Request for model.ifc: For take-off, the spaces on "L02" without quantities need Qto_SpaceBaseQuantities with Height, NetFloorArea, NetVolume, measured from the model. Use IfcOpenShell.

First a look at what the model holds.

```python
import ifcopenshell
import ifcopenshell.util.element
import ifcopenshell.util.unit

model = ifcopenshell.open("model.ifc")
print(model.schema)
for unit_type in ("LENGTHUNIT", "AREAUNIT", "VOLUMEUNIT"):
    print(unit_type, ifcopenshell.util.unit.calculate_unit_scale(model, unit_type))
storey = next(s for s in model.by_type("IfcBuildingStorey") if s.Name == "L02")
spaces = [e for e in ifcopenshell.util.element.get_decomposition(storey) if e.is_a("IfcSpace")]
for e in sorted(spaces, key=lambda e: e.id()):
    print(e.id(), e.is_a(), e.Name, list(ifcopenshell.util.element.get_psets(e, qtos_only=True)), sep=" | ")
```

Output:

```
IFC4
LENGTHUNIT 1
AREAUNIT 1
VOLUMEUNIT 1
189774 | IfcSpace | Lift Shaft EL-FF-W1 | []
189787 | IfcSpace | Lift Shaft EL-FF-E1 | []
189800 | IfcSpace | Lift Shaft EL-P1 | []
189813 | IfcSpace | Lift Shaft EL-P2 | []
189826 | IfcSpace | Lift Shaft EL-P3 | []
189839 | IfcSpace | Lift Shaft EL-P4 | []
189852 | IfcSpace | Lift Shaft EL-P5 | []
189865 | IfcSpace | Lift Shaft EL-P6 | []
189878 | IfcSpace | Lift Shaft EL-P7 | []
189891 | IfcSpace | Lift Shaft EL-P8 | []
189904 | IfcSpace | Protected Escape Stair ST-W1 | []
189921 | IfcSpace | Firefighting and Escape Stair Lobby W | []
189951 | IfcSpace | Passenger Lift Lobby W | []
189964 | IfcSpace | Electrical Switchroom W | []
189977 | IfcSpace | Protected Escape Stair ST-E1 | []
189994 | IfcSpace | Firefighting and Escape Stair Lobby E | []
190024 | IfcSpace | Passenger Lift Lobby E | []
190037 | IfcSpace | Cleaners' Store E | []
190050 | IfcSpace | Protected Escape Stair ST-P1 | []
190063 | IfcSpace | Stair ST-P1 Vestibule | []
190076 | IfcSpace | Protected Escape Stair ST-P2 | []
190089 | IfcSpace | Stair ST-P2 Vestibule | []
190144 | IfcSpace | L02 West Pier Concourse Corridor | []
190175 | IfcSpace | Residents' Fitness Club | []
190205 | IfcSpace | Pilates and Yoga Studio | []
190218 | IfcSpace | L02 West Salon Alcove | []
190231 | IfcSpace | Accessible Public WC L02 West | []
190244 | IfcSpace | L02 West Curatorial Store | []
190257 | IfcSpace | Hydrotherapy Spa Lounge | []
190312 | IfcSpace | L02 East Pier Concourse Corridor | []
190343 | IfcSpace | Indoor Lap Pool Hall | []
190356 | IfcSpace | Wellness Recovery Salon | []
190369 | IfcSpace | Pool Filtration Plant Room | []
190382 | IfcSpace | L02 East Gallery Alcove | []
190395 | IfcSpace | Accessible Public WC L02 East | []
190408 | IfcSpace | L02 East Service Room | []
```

```python
import ifcopenshell
import ifcopenshell.api.pset
import ifcopenshell.geom
import ifcopenshell.util.element
import ifcopenshell.util.shape
import ifcopenshell.util.unit

model = ifcopenshell.open("model.ifc")
unit_scale = ifcopenshell.util.unit.calculate_unit_scale(model)
area_scale = ifcopenshell.util.unit.calculate_unit_scale(model, "AREAUNIT")
volume_scale = ifcopenshell.util.unit.calculate_unit_scale(model, "VOLUMEUNIT")
settings = ifcopenshell.geom.settings()

storey = next(s for s in model.by_type("IfcBuildingStorey") if s.Name == "L02")
spaces = [e for e in ifcopenshell.util.element.get_decomposition(storey) if e.is_a("IfcSpace")]

for e in sorted(spaces, key=lambda e: e.id()):
    if ifcopenshell.util.element.get_psets(e, qtos_only=True, should_inherit=False):
        continue
    # Geometry comes back in metres, in the element's own axes.
    shape = ifcopenshell.geom.create_shape(settings, e)
    values = {
        "Height": ifcopenshell.util.shape.get_z(shape.geometry) / unit_scale,
        "NetFloorArea": ifcopenshell.util.shape.get_footprint_area(shape.geometry) / area_scale,
        "NetVolume": ifcopenshell.util.shape.get_volume(shape.geometry) / volume_scale,
    }
    qto = ifcopenshell.api.pset.add_qto(model, product=e, name="Qto_SpaceBaseQuantities")
    ifcopenshell.api.pset.edit_qto(model, qto=qto, properties=values)
    print(e.id(), {k: round(v, 3) for k, v in values.items()})

model.write("model_edited.ifc")
```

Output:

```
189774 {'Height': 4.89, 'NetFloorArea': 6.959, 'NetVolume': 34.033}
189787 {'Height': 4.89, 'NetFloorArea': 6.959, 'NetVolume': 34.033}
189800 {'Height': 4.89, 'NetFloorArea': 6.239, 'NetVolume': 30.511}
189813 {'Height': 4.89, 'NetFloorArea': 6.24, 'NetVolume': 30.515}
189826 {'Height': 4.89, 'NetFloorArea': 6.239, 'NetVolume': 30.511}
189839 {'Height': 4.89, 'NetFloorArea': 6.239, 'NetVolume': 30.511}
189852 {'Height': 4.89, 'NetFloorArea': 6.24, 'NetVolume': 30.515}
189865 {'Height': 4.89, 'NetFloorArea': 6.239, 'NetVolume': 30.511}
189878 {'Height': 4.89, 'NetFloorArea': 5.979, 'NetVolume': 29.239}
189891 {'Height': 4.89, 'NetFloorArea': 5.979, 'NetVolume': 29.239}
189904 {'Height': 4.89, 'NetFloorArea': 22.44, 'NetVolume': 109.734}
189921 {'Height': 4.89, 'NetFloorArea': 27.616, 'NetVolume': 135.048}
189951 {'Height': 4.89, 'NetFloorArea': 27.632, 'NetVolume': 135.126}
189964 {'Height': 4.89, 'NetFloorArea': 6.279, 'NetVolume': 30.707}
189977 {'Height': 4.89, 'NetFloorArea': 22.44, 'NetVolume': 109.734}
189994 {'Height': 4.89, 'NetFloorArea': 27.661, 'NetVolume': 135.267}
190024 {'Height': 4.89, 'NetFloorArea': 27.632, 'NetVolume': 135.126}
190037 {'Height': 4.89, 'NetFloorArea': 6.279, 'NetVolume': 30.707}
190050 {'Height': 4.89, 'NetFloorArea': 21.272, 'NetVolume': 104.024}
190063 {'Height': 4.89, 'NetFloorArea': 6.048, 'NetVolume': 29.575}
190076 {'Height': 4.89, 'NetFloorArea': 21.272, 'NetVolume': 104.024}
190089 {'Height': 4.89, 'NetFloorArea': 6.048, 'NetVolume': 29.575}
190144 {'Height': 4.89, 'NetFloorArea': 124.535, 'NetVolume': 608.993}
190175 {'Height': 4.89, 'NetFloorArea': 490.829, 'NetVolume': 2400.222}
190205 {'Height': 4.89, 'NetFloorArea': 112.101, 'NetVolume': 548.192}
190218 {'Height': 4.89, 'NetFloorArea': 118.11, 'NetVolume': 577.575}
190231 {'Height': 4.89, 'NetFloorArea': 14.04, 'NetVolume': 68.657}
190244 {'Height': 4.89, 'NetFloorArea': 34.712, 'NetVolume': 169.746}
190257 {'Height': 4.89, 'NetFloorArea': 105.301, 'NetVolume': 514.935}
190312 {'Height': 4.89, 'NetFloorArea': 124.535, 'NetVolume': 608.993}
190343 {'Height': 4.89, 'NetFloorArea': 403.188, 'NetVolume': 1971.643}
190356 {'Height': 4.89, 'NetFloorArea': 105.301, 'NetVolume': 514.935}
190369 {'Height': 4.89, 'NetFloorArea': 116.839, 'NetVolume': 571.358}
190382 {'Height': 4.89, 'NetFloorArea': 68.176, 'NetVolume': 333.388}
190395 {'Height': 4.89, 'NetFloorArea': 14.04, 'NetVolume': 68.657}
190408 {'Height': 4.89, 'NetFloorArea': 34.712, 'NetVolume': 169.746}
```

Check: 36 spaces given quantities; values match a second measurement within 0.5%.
